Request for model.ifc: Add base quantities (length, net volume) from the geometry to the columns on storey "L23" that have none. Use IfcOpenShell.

First a look at what the model holds.

```python
import ifcopenshell
import ifcopenshell.util.element
import ifcopenshell.util.unit

model = ifcopenshell.open("model.ifc")
print(model.schema)
for unit_type in ("LENGTHUNIT", "AREAUNIT", "VOLUMEUNIT"):
    print(unit_type, ifcopenshell.util.unit.calculate_unit_scale(model, unit_type))
storey = next(s for s in model.by_type("IfcBuildingStorey") if s.Name == "L23")
columns = [e for e in ifcopenshell.util.element.get_decomposition(storey) if e.is_a("IfcColumn")]
for e in sorted(columns, key=lambda e: e.id()):
    print(e.id(), e.is_a(), e.Name, list(ifcopenshell.util.element.get_psets(e, qtos_only=True)), sep=" | ")
```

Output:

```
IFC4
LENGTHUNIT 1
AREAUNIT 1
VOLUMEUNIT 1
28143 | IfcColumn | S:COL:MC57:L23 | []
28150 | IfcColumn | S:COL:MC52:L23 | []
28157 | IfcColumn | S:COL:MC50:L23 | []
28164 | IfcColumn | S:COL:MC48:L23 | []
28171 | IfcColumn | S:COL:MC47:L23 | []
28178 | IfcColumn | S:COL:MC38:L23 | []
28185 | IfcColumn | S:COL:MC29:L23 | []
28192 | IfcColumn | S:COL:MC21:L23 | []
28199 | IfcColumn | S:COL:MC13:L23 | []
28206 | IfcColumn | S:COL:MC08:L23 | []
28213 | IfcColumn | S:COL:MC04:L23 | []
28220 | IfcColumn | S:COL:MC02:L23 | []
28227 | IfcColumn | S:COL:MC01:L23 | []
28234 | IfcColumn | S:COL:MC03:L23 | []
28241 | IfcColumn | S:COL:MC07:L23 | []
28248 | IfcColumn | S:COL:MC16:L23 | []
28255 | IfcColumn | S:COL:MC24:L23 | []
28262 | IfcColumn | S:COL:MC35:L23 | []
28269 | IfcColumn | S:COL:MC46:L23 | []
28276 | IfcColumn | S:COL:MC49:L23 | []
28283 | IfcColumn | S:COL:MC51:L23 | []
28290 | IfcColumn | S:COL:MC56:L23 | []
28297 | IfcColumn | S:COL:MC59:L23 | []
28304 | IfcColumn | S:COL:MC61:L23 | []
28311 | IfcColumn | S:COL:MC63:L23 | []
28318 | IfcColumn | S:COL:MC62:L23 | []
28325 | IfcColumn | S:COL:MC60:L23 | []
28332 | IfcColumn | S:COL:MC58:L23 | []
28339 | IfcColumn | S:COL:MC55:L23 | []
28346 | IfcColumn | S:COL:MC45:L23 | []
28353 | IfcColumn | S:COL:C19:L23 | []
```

```python
import ifcopenshell
import ifcopenshell.api.pset
import ifcopenshell.geom
import ifcopenshell.util.element
import ifcopenshell.util.shape
import ifcopenshell.util.unit

model = ifcopenshell.open("model.ifc")
unit_scale = ifcopenshell.util.unit.calculate_unit_scale(model)
volume_scale = ifcopenshell.util.unit.calculate_unit_scale(model, "VOLUMEUNIT")
settings = ifcopenshell.geom.settings()

storey = next(s for s in model.by_type("IfcBuildingStorey") if s.Name == "L23")
columns = [e for e in ifcopenshell.util.element.get_decomposition(storey) if e.is_a("IfcColumn")]

for e in sorted(columns, key=lambda e: e.id()):
    if ifcopenshell.util.element.get_psets(e, qtos_only=True, should_inherit=False):
        continue
    # Geometry comes back in metres, in the element's own axes.
    shape = ifcopenshell.geom.create_shape(settings, e)
    values = {
        "Length": ifcopenshell.util.shape.get_z(shape.geometry) / unit_scale,
        "NetVolume": ifcopenshell.util.shape.get_volume(shape.geometry) / volume_scale,
    }
    qto = ifcopenshell.api.pset.add_qto(model, product=e, name="Qto_ColumnBaseQuantities")
    ifcopenshell.api.pset.edit_qto(model, qto=qto, properties=values)
    print(e.id(), {k: round(v, 3) for k, v in values.items()})

model.write("model_rev.ifc")
```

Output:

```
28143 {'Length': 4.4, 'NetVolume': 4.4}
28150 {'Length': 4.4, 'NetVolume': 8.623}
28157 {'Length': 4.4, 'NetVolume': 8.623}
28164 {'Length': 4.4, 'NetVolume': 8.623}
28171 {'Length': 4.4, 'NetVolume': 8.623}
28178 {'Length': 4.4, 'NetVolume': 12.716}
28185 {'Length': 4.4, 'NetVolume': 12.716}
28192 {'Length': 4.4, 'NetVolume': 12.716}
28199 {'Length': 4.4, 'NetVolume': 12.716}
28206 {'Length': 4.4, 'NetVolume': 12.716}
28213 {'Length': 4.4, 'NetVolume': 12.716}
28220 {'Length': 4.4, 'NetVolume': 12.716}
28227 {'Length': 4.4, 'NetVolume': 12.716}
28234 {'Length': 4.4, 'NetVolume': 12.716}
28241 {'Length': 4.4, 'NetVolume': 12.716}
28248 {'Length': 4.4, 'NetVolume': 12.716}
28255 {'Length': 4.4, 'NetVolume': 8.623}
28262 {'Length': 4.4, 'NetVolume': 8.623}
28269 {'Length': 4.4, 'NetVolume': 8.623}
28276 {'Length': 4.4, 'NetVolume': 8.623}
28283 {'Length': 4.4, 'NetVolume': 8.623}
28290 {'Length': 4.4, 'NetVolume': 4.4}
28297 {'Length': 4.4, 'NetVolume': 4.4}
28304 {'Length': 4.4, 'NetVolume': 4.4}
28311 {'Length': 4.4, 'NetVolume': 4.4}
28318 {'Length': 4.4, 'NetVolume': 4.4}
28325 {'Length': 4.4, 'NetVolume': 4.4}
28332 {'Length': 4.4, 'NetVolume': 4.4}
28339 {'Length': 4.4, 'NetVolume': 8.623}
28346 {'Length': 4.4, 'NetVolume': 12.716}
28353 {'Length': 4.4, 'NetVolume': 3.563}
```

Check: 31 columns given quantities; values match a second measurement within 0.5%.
